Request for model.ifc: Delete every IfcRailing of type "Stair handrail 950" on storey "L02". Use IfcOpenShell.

First a look at what the model holds.

```python
import ifcopenshell
import ifcopenshell.util.element

model = ifcopenshell.open("model.ifc")
print(model.schema)
storey = next(s for s in model.by_type("IfcBuildingStorey") if s.Name == "L02")
railings = [e for e in ifcopenshell.util.element.get_decomposition(storey) if e.is_a("IfcRailing")]
seen = {}
for e in railings:
    element_type = ifcopenshell.util.element.get_type(e)
    name = element_type.Name if element_type not in (None, e) else None
    seen[name] = seen.get(name, 0) + 1
for name, count in sorted(seen.items(), key=str):
    print(count, "x", name)
```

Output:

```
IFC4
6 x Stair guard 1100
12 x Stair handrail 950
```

```python
import ifcopenshell
import ifcopenshell.api.root
import ifcopenshell.util.element

model = ifcopenshell.open("model.ifc")

storey = next(s for s in model.by_type("IfcBuildingStorey") if s.Name == "L02")
railings = [e for e in ifcopenshell.util.element.get_decomposition(storey) if e.is_a("IfcRailing")]
targets = [e for e in railings if (t := ifcopenshell.util.element.get_type(e)) not in (None, e) and t.Name == "Stair handrail 950"]

for e in targets:
    ifcopenshell.api.root.remove_product(model, product=e)
print(len(targets), "removed")

model.write("model-out.ifc")
```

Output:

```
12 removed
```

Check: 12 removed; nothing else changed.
